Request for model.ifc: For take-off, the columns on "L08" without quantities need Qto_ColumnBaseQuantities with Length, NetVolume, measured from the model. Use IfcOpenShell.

First a look at what the model holds.

```python
import ifcopenshell
import ifcopenshell.util.element
import ifcopenshell.util.unit

model = ifcopenshell.open("model.ifc")
print(model.schema)
for unit_type in ("LENGTHUNIT", "AREAUNIT", "VOLUMEUNIT"):
    print(unit_type, ifcopenshell.util.unit.calculate_unit_scale(model, unit_type))
storey = next(s for s in model.by_type("IfcBuildingStorey") if s.Name == "L08")
columns = [e for e in ifcopenshell.util.element.get_decomposition(storey) if e.is_a("IfcColumn")]
for e in sorted(columns, key=lambda e: e.id()):
    print(e.id(), e.is_a(), e.Name, list(ifcopenshell.util.element.get_psets(e, qtos_only=True)), sep=" | ")
```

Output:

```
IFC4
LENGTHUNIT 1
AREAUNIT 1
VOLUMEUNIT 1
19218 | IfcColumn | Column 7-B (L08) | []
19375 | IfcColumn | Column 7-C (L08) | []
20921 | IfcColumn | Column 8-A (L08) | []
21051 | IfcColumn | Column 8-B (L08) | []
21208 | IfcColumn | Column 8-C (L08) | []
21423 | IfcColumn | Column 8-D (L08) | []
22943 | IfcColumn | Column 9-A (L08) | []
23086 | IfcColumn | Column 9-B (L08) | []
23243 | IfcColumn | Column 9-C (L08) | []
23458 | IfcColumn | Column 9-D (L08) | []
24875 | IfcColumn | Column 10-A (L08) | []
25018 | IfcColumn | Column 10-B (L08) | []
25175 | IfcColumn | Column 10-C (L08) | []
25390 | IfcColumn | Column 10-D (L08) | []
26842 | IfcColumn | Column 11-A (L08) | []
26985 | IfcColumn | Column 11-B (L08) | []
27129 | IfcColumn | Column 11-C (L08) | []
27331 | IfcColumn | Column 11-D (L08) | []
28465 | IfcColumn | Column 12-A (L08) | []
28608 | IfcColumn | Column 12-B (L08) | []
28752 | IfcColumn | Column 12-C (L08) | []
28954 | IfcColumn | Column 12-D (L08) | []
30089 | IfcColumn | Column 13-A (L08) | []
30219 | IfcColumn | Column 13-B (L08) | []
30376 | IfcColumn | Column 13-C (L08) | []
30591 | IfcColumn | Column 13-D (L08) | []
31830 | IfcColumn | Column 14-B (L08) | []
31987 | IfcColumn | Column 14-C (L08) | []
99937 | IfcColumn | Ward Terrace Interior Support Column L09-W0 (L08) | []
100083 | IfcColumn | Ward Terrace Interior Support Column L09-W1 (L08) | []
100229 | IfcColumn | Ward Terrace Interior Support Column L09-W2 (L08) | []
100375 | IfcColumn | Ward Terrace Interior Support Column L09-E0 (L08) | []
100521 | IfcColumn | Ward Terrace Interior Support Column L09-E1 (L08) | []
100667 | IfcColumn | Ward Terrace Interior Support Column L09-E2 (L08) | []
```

```python
import ifcopenshell
import ifcopenshell.api.pset
import ifcopenshell.geom
import ifcopenshell.util.element
import ifcopenshell.util.shape
import ifcopenshell.util.unit

model = ifcopenshell.open("model.ifc")
unit_scale = ifcopenshell.util.unit.calculate_unit_scale(model)
volume_scale = ifcopenshell.util.unit.calculate_unit_scale(model, "VOLUMEUNIT")
settings = ifcopenshell.geom.settings()

storey = next(s for s in model.by_type("IfcBuildingStorey") if s.Name == "L08")
columns = [e for e in ifcopenshell.util.element.get_decomposition(storey) if e.is_a("IfcColumn")]

for e in sorted(columns, key=lambda e: e.id()):
    if ifcopenshell.util.element.get_psets(e, qtos_only=True, should_inherit=False):
        continue
    # Geometry comes back in metres, in the element's own axes.
    shape = ifcopenshell.geom.create_shape(settings, e)
    values = {
        "Length": ifcopenshell.util.shape.get_z(shape.geometry) / unit_scale,
        "NetVolume": ifcopenshell.util.shape.get_volume(shape.geometry) / volume_scale,
    }
    qto = ifcopenshell.api.pset.add_qto(model, product=e, name="Qto_ColumnBaseQuantities")
    ifcopenshell.api.pset.edit_qto(model, qto=qto, properties=values)
    print(e.id(), {k: round(v, 3) for k, v in values.items()})

model.write("model_rev.ifc")
```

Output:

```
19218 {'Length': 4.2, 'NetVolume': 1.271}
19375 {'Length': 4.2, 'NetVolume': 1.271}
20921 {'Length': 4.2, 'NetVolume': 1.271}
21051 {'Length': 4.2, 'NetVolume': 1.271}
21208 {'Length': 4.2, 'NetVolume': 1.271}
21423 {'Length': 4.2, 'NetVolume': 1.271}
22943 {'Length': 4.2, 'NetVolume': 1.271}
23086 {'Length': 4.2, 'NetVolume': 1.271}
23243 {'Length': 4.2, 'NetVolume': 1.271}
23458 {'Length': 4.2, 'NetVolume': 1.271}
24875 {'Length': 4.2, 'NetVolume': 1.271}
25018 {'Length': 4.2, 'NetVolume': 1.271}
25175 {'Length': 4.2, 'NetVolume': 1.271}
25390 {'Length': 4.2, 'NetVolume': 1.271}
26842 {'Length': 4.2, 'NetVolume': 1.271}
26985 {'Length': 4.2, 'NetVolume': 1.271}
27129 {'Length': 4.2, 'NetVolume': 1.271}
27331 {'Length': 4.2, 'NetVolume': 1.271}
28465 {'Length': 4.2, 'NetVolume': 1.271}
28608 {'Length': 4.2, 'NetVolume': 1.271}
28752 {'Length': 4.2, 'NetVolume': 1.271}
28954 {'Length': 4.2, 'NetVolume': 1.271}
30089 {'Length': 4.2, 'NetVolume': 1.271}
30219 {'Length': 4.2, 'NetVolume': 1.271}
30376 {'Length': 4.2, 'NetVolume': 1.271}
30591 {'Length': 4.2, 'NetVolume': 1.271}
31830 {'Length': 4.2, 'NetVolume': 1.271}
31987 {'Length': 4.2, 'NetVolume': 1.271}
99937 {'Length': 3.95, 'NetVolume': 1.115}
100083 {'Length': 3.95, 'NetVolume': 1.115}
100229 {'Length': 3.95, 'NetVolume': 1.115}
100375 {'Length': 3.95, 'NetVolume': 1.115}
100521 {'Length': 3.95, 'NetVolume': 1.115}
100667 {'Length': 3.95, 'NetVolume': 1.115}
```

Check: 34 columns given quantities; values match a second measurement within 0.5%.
